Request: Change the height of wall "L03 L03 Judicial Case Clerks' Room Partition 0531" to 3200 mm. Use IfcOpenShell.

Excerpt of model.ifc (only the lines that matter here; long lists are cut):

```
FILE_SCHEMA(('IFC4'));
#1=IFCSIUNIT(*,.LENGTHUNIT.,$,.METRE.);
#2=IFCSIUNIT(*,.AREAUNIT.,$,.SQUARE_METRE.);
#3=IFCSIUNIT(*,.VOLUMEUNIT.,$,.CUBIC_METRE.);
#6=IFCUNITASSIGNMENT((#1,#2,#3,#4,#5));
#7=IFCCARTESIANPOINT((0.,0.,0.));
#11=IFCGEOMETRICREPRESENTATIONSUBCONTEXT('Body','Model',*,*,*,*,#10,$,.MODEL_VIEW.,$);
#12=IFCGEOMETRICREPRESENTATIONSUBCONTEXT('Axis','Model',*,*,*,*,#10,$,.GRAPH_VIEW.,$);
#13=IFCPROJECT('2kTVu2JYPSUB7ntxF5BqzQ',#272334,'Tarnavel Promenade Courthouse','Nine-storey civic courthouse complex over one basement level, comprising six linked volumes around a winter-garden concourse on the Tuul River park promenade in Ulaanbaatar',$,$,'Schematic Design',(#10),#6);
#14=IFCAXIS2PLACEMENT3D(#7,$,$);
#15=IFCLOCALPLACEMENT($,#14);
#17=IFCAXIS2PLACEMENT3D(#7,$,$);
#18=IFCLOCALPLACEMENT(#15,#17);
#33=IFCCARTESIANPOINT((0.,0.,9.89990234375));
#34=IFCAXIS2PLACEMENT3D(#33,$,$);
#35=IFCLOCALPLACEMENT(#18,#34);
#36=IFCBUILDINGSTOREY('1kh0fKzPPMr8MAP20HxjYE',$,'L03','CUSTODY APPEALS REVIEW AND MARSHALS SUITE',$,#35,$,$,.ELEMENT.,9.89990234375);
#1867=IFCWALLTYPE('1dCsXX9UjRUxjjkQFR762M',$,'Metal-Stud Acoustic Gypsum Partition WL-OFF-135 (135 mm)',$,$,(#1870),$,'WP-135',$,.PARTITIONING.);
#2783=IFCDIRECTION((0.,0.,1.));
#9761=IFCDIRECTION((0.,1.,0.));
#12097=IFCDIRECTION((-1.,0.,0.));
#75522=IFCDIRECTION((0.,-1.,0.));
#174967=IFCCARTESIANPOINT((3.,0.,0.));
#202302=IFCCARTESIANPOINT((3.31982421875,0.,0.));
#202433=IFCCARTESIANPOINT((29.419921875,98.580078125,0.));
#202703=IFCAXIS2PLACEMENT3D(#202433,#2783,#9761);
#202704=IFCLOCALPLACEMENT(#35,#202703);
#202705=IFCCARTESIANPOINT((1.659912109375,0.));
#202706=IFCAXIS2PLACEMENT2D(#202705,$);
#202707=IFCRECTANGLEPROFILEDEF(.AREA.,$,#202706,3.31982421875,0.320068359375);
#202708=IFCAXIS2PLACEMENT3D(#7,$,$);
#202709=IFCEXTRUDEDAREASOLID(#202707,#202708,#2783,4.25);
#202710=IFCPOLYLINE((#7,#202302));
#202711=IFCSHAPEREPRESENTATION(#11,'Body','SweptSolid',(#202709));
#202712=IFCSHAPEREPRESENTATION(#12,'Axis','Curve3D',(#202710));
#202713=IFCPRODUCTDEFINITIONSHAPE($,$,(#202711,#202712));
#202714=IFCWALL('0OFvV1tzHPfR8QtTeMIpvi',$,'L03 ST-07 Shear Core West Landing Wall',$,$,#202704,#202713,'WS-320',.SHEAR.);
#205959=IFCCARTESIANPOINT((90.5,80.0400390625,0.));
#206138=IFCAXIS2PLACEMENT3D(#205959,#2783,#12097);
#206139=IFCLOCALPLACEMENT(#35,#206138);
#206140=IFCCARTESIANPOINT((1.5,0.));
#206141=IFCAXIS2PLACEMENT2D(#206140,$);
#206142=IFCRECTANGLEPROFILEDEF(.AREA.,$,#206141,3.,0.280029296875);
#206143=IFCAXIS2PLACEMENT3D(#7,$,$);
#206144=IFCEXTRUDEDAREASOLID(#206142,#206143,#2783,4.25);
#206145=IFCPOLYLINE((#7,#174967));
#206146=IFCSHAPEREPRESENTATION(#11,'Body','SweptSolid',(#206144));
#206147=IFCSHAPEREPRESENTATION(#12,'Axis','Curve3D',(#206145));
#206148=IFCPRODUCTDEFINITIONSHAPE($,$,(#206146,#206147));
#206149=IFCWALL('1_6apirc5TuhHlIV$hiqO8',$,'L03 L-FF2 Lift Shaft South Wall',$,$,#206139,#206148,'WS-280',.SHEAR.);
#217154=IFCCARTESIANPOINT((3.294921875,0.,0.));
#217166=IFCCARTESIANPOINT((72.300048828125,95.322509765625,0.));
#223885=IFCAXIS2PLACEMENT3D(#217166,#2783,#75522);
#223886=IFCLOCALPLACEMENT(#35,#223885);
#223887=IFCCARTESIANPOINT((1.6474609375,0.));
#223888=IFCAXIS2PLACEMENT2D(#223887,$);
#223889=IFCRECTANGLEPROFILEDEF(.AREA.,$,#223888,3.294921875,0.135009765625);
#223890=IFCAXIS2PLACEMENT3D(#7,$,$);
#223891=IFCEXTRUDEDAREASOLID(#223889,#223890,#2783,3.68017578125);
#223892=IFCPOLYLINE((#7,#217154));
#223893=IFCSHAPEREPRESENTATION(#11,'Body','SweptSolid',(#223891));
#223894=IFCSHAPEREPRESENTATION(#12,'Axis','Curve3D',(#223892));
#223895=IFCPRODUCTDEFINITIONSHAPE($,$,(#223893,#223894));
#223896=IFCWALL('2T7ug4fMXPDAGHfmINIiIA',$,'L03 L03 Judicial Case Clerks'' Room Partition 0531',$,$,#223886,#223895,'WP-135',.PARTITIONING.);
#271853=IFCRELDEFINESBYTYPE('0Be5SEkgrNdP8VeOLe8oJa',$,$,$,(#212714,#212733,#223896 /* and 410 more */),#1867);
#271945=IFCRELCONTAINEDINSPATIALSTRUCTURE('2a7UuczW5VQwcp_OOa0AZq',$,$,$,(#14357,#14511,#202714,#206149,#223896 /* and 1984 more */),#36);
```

```python
import ifcopenshell
import ifcopenshell.geom
import ifcopenshell.util.representation
import ifcopenshell.util.shape

model = ifcopenshell.open("model.ifc")
settings = ifcopenshell.geom.settings()


def volume(element):
    """Net volume in cubic metres, openings subtracted."""
    shape = ifcopenshell.geom.create_shape(settings, element)
    return ifcopenshell.util.shape.get_volume(shape.geometry)


wall = model.by_guid("2T7ug4fMXPDAGHfmINIiIA")
before = volume(wall)

body = ifcopenshell.util.representation.get_representation(wall, "Model", "Body")
solid = body.Items[0]
old_height = solid.Depth
solid.Depth = 3.2
after = volume(wall)

print(f"height {old_height:g} -> {solid.Depth:g}, volume {before:.3f} -> {after:.3f} m3")

model.write("model_updated.ifc")
```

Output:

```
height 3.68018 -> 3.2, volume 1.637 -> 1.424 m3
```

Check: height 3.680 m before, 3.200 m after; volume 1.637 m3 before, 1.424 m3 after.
